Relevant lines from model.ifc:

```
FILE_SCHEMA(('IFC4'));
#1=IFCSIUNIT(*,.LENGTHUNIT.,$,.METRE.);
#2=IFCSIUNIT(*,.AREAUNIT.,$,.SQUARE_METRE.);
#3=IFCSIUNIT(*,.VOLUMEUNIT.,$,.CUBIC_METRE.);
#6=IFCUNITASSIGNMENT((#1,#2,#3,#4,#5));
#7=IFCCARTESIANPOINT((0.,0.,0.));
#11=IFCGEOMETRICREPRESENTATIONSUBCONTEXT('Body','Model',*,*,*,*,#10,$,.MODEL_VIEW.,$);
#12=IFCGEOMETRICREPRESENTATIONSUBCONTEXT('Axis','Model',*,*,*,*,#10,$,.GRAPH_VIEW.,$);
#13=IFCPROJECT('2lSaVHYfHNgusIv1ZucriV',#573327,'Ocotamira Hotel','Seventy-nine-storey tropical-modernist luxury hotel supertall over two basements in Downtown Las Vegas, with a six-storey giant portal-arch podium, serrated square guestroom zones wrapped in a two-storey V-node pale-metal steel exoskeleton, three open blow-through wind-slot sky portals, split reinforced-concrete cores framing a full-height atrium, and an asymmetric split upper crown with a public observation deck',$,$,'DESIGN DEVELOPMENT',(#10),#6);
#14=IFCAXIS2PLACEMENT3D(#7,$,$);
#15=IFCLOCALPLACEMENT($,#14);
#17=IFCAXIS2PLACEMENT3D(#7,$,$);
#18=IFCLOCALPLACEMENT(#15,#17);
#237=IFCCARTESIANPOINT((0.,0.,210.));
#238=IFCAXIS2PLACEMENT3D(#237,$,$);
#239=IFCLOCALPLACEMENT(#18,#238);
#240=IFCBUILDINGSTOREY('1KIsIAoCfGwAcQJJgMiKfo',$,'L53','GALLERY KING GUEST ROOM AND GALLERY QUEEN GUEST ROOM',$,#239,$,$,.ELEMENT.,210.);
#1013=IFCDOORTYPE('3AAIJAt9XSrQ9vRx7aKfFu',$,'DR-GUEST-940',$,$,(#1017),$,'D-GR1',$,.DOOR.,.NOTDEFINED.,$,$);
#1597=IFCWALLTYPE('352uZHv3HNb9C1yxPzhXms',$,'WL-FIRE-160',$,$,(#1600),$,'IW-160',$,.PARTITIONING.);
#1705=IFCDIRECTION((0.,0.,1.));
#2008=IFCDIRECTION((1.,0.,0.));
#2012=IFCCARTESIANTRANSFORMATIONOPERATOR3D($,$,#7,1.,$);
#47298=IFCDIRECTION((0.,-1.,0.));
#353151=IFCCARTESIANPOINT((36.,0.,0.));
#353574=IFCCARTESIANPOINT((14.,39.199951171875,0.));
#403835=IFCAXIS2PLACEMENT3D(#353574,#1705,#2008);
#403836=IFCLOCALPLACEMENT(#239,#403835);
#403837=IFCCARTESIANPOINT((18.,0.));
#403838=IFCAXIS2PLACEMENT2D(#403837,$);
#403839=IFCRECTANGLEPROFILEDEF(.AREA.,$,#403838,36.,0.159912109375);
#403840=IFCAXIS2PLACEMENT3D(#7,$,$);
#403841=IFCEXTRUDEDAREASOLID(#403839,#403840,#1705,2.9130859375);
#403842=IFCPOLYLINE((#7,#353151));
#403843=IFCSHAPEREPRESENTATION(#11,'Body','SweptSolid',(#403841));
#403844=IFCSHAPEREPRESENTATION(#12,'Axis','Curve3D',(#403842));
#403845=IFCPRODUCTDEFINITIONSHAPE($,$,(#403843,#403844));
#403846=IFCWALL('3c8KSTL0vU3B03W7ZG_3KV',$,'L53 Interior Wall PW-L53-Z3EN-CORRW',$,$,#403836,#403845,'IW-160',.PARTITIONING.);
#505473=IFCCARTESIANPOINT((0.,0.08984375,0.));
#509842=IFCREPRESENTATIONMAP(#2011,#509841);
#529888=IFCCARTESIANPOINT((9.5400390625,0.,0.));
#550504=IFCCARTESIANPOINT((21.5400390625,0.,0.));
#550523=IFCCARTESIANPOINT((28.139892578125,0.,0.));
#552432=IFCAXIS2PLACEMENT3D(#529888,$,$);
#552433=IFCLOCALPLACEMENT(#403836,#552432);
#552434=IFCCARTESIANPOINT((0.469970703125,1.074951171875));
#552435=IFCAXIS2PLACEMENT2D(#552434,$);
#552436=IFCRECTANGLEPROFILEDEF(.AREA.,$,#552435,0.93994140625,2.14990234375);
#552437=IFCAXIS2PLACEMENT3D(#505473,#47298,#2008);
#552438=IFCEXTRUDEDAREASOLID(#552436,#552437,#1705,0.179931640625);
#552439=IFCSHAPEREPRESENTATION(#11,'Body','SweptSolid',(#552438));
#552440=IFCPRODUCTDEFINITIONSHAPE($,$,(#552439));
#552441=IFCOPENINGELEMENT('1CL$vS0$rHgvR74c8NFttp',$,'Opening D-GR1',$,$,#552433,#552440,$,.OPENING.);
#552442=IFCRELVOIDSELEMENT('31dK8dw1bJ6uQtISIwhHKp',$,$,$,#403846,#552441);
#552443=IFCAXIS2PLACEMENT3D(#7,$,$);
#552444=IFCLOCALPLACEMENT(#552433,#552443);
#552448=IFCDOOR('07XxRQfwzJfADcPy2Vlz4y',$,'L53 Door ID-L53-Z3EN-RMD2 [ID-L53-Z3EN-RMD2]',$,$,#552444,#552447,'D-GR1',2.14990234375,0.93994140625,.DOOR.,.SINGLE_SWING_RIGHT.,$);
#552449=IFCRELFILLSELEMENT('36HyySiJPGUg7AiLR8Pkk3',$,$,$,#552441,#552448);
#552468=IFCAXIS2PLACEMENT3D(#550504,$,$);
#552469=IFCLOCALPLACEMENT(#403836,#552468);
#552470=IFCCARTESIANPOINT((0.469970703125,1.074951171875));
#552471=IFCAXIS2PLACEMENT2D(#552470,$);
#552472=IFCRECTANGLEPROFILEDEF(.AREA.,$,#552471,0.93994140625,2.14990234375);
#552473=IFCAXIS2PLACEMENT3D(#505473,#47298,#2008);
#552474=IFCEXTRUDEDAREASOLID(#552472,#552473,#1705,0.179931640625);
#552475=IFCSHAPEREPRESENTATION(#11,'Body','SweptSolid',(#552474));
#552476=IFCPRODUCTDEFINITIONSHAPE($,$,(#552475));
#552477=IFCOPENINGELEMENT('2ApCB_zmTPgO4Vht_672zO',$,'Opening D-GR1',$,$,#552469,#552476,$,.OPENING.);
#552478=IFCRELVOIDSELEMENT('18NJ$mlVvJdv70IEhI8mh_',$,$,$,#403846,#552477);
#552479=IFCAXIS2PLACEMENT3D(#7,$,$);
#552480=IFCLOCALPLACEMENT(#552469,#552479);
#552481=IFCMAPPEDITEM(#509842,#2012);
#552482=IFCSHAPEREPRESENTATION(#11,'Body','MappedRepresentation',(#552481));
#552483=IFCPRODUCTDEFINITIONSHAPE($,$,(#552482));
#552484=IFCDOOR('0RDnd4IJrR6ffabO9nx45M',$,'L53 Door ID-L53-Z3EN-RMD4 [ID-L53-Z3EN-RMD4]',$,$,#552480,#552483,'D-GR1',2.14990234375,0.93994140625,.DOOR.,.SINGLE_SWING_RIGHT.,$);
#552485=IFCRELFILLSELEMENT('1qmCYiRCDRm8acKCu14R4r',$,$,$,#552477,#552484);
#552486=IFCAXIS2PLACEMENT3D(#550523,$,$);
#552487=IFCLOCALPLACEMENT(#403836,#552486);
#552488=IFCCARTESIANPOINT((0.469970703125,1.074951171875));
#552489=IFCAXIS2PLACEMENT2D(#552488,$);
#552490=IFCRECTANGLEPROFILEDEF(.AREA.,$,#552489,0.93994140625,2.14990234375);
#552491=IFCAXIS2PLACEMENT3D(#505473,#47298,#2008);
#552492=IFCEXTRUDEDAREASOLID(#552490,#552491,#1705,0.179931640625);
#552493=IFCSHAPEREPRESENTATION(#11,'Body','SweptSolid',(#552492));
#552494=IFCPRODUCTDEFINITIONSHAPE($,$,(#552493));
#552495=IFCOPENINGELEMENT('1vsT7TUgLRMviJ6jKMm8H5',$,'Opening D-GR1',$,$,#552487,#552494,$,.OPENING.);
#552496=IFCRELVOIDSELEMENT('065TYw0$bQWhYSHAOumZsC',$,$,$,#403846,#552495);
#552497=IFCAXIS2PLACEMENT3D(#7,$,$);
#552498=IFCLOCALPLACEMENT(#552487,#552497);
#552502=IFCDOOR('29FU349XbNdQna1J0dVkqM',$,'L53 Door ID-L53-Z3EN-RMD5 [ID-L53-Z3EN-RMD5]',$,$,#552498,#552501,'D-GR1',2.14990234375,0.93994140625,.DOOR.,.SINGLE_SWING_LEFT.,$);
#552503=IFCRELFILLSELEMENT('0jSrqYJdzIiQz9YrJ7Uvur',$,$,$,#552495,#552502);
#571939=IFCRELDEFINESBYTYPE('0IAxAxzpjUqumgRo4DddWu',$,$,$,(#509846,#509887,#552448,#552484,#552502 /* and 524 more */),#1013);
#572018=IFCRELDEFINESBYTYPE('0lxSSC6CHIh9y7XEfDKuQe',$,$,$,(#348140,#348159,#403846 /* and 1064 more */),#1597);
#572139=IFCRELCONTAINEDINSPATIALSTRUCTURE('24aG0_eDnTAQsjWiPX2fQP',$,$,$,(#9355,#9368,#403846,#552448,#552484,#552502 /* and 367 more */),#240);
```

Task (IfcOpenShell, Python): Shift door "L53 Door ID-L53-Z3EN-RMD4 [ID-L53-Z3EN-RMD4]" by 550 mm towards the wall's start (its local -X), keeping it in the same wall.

```python
import ifcopenshell
import ifcopenshell.api.geometry
import ifcopenshell.util.placement

model = ifcopenshell.open("model.ifc")

door = model.by_guid("0RDnd4IJrR6ffabO9nx45M")
opening = door.FillsVoids[0].RelatingOpeningElement
wall = opening.VoidsElements[0].RelatingBuildingElement

wall_matrix = ifcopenshell.util.placement.get_local_placement(wall.ObjectPlacement)
shift = wall_matrix[:3, 0] * -0.55
before = ifcopenshell.util.placement.get_local_placement(door.ObjectPlacement)[:3, 3].copy()

# The door is placed relative to its opening, so it follows when the opening moves.
matrix = ifcopenshell.util.placement.get_local_placement(opening.ObjectPlacement)
matrix[:3, 3] += shift
ifcopenshell.api.geometry.edit_object_placement(
    model, product=opening, matrix=matrix, is_si=False, should_transform_children=True
)

after = ifcopenshell.util.placement.get_local_placement(door.ObjectPlacement)[:3, 3]
print("door moved by", (after - before).round(3) + 0.0)

model.write("model_updated.ifc")
```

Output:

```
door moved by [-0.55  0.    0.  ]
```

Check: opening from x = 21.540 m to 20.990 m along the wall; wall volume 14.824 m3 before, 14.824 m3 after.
